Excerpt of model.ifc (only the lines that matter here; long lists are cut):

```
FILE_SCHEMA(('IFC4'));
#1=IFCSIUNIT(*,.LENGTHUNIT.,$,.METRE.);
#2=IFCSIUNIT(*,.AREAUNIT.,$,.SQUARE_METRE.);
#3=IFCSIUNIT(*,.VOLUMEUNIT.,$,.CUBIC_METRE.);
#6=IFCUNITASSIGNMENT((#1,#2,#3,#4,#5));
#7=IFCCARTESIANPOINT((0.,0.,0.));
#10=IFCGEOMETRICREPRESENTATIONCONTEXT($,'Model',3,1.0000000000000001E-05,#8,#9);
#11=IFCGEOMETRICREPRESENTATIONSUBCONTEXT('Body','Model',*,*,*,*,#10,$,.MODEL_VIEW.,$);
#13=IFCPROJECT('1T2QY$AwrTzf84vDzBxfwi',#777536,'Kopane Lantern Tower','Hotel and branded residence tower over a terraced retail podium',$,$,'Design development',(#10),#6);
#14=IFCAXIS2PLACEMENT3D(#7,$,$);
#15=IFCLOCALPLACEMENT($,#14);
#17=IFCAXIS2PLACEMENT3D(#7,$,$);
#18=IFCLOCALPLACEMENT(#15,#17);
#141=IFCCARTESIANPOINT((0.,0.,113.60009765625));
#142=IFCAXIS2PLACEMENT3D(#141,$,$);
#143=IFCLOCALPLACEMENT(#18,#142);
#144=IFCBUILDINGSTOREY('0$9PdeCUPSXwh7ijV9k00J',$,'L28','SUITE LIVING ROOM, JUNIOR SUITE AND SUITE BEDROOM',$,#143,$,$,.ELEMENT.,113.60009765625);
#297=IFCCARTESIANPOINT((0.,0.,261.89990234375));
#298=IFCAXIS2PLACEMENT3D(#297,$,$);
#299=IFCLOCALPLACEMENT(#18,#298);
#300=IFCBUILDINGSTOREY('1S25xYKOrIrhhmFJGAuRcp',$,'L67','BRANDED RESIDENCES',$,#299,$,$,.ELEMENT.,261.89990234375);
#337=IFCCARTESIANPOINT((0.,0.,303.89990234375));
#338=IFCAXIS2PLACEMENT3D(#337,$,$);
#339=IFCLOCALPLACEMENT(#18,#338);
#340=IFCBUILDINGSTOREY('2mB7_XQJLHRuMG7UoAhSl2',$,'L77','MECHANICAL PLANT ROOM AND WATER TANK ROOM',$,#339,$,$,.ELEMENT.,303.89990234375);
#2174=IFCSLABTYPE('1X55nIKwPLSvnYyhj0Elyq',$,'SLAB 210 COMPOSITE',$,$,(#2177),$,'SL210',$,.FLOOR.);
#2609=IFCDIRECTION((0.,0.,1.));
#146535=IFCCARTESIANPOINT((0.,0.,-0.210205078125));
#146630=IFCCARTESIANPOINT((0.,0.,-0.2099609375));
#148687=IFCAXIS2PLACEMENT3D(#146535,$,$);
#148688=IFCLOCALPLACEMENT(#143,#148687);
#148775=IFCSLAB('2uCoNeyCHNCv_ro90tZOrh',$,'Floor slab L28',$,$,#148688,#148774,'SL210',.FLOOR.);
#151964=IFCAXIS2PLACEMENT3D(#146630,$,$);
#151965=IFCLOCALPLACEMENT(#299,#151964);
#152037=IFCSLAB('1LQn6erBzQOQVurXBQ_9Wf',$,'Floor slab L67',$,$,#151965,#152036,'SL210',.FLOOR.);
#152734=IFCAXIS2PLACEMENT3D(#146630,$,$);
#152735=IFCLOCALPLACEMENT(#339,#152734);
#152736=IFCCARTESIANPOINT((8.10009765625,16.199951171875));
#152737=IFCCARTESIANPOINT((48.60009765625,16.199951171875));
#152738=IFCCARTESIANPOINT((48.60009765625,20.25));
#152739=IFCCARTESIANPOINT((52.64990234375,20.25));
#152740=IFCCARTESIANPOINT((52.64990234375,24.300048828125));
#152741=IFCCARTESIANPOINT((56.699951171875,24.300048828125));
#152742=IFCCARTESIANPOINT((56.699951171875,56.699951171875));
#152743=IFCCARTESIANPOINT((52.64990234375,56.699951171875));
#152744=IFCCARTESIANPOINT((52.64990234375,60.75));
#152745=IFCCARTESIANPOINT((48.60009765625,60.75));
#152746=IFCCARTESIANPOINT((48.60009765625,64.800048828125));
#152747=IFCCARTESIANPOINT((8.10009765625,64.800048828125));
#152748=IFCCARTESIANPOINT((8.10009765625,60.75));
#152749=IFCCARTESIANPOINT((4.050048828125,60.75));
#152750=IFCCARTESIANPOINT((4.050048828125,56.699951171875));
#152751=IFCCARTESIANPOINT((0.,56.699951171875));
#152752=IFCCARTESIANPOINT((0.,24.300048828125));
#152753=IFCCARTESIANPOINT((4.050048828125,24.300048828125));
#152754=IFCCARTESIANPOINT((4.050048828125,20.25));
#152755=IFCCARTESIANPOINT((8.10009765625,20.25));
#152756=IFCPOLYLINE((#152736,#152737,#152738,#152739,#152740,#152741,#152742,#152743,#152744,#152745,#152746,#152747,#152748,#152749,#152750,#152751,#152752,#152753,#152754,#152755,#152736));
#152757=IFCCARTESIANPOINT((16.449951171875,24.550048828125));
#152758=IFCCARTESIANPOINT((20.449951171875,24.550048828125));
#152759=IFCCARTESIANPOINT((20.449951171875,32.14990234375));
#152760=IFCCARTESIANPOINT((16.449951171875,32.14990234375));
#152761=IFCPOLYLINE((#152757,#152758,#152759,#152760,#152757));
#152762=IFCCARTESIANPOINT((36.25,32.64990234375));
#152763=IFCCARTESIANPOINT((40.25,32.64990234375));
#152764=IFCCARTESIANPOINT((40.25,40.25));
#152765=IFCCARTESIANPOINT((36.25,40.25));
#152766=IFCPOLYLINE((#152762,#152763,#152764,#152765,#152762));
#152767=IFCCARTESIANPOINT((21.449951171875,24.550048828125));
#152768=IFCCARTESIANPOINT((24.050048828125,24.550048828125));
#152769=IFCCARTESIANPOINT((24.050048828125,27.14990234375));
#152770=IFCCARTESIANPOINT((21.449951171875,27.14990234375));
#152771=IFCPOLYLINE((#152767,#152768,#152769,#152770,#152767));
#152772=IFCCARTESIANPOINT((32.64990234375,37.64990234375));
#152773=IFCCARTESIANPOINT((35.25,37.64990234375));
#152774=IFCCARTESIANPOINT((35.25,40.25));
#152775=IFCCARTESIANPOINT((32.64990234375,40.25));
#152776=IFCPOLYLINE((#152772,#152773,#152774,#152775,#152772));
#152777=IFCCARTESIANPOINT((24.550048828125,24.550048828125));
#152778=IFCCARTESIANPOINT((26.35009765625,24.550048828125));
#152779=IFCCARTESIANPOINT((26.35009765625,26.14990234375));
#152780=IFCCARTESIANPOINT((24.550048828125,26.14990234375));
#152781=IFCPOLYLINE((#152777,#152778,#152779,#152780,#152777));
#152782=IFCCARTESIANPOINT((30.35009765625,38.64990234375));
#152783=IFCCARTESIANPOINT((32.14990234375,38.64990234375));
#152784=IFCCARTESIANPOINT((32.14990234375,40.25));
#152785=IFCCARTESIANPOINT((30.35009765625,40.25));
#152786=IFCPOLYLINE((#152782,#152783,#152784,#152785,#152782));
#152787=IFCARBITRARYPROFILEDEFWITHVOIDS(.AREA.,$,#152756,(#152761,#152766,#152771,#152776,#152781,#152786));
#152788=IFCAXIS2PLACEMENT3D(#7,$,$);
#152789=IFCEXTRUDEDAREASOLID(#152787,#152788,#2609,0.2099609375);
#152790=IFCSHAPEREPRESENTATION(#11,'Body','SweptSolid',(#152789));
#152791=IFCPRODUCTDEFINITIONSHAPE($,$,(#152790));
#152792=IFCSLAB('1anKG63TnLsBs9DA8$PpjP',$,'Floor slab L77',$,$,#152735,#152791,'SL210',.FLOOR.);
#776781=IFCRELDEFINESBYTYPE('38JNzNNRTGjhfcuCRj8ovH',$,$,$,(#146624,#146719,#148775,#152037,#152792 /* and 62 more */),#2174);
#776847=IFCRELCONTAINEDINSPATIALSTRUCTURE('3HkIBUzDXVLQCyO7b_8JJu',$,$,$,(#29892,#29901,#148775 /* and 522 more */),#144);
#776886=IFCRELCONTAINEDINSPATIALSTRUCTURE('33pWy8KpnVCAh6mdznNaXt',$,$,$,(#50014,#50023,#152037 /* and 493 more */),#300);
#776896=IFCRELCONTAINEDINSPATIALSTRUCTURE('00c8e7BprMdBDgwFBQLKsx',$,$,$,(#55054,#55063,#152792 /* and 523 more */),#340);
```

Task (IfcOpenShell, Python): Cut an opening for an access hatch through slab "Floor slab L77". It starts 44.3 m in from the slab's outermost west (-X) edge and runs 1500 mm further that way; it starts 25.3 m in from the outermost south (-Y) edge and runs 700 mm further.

```python
import numpy as np
import ifcopenshell
import ifcopenshell.api.feature
import ifcopenshell.api.geometry
import ifcopenshell.api.root
import ifcopenshell.geom
import ifcopenshell.util.placement
import ifcopenshell.util.representation
import ifcopenshell.util.shape
import ifcopenshell.util.unit

model = ifcopenshell.open("model.ifc")
unit_scale = ifcopenshell.util.unit.calculate_unit_scale(model)
settings = ifcopenshell.geom.settings()


def volume(element):
    """Net volume in cubic metres, openings subtracted."""
    shape = ifcopenshell.geom.create_shape(settings, element)
    return ifcopenshell.util.shape.get_volume(shape.geometry)


slab = model.by_guid("1anKG63TnLsBs9DA8$PpjP")
before = volume(slab)

# Extent in the slab's own axes, in metres. The edges named are its -X and -Y sides.
slab_shape = ifcopenshell.geom.create_shape(settings, slab)
vertices = ifcopenshell.util.shape.get_vertices(slab_shape.geometry)
x_min, y_min, bottom = vertices.min(axis=0)
top = vertices[:, 2].max()

opening = ifcopenshell.api.root.create_entity(model, ifc_class="IfcOpeningElement", name="Access hatch opening", predefined_type="OPENING")
context = ifcopenshell.util.representation.get_context(model, "Model", "Body", "MODEL_VIEW")
width, depth = 1.5, 0.7
outline = [(0.0, 0.0), (width, 0.0), (width, depth), (0.0, depth), (0.0, 0.0)]
# Overshoot both faces by 50 mm so the cut is clean.
shape = ifcopenshell.api.geometry.add_slab_representation(
    model, context=context, depth=top - bottom + 0.1, polyline=outline
)
ifcopenshell.api.geometry.assign_representation(model, product=opening, representation=shape)

matrix = ifcopenshell.util.placement.get_local_placement(slab.ObjectPlacement)
matrix[:, 3] = matrix @ np.append(np.array([x_min + 44.3, y_min + 25.3, bottom - 0.05]) / unit_scale, 1.0)
ifcopenshell.api.geometry.edit_object_placement(model, product=opening, matrix=matrix, is_si=False)
ifcopenshell.api.feature.add_feature(model, feature=opening, element=slab)

after = volume(slab)

print(f"slab volume {before:.3f} -> {after:.3f} m3")

model.write("model_v2.ifc")
```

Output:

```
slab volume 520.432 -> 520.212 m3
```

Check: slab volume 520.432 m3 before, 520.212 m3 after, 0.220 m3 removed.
